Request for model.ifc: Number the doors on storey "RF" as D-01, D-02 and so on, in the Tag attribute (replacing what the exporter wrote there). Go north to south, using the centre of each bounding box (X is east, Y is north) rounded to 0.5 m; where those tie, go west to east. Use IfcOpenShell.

First a look at what the model holds.

```python
import ifcopenshell
import ifcopenshell.util.element
import ifcopenshell.util.placement

model = ifcopenshell.open("model.ifc")
print(model.schema)
storey = next(s for s in model.by_type("IfcBuildingStorey") if s.Name == "RF")
doors = [e for e in ifcopenshell.util.element.get_decomposition(storey) if e.is_a("IfcDoor")]
for e in sorted(doors, key=lambda e: e.id()):
    origin = ifcopenshell.util.placement.get_local_placement(e.ObjectPlacement)[:3, 3]
    print(e.id(), e.Tag, e.Name, origin.round(2) + 0.0, sep=" | ")
```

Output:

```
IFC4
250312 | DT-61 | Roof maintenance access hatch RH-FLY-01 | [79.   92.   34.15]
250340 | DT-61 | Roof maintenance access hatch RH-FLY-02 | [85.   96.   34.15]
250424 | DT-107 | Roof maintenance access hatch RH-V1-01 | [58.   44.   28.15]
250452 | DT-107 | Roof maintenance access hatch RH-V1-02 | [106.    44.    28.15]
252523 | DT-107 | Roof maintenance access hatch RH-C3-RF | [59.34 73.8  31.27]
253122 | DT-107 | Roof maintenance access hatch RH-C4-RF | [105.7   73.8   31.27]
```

```python
import ifcopenshell
import ifcopenshell.geom
import ifcopenshell.util.element
import ifcopenshell.util.shape

model = ifcopenshell.open("model.ifc")
settings = ifcopenshell.geom.settings()
settings.set("use-world-coords", True)


def centre(element):
    shape = ifcopenshell.geom.create_shape(settings, element)
    return ifcopenshell.util.shape.get_bbox_centroid(shape.geometry)


storey = next(s for s in model.by_type("IfcBuildingStorey") if s.Name == "RF")
doors = [e for e in ifcopenshell.util.element.get_decomposition(storey) if e.is_a("IfcDoor")]

# Insertion points can sit at a corner or the storey origin, so sort by the geometry (in metres).
centres = {e: centre(e) for e in doors}
doors.sort(key=lambda e: (-round(centres[e][1] / 0.5), centres[e][0]))

for i, e in enumerate(doors, start=1):
    number = f"D-{i:02d}"
    e.Tag = number
    print(e.id(), number)

model.write("model_rev.ifc")
```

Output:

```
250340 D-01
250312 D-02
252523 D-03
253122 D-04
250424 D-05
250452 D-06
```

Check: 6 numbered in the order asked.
